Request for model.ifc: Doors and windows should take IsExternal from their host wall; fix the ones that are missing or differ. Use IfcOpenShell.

First a look at what the model holds.

```python
import ifcopenshell
import ifcopenshell.util.element

model = ifcopenshell.open("model.ifc")
print(model.schema)
seen = {}
for e in model.by_type("IfcDoor") + model.by_type("IfcWindow"):
    if not e.FillsVoids:
        continue
    host = e.FillsVoids[0].RelatingOpeningElement.VoidsElements[0].RelatingBuildingElement
    own = ifcopenshell.util.element.get_pset(e, f"Pset_{e.is_a()[3:].removesuffix('StandardCase')}Common", "IsExternal")
    wall = ifcopenshell.util.element.get_pset(host, "Pset_WallCommon", "IsExternal")
    seen[e.is_a(), own, wall] = seen.get((e.is_a(), own, wall), 0) + 1
for (cls, own, wall), count in sorted(seen.items(), key=str):
    print(count, cls, "IsExternal:", own, "| host wall:", wall)
```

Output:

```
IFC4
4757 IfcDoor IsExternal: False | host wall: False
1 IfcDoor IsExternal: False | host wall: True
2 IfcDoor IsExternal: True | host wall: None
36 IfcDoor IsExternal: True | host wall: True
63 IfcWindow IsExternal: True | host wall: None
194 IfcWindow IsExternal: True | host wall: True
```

```python
import ifcopenshell
import ifcopenshell.api.pset
import ifcopenshell.util.element

model = ifcopenshell.open("model.ifc")

count = 0
for ifc_class, pset_name in (("IfcDoor", "Pset_DoorCommon"), ("IfcWindow", "Pset_WindowCommon")):
    for e in model.by_type(ifc_class):
        if not e.FillsVoids:
            continue
        host = e.FillsVoids[0].RelatingOpeningElement.VoidsElements[0].RelatingBuildingElement
        external = ifcopenshell.util.element.get_pset(host, "Pset_WallCommon", "IsExternal")
        if external is None or ifcopenshell.util.element.get_pset(e, pset_name, "IsExternal") == external:
            continue
        pset = ifcopenshell.api.pset.add_pset(model, product=e, name=pset_name)
        ifcopenshell.api.pset.edit_pset(model, pset=pset, properties={"IsExternal": external})
        count += 1

print(count, "updated")

model.write("model_updated.ifc")
```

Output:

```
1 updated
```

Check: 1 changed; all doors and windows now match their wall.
